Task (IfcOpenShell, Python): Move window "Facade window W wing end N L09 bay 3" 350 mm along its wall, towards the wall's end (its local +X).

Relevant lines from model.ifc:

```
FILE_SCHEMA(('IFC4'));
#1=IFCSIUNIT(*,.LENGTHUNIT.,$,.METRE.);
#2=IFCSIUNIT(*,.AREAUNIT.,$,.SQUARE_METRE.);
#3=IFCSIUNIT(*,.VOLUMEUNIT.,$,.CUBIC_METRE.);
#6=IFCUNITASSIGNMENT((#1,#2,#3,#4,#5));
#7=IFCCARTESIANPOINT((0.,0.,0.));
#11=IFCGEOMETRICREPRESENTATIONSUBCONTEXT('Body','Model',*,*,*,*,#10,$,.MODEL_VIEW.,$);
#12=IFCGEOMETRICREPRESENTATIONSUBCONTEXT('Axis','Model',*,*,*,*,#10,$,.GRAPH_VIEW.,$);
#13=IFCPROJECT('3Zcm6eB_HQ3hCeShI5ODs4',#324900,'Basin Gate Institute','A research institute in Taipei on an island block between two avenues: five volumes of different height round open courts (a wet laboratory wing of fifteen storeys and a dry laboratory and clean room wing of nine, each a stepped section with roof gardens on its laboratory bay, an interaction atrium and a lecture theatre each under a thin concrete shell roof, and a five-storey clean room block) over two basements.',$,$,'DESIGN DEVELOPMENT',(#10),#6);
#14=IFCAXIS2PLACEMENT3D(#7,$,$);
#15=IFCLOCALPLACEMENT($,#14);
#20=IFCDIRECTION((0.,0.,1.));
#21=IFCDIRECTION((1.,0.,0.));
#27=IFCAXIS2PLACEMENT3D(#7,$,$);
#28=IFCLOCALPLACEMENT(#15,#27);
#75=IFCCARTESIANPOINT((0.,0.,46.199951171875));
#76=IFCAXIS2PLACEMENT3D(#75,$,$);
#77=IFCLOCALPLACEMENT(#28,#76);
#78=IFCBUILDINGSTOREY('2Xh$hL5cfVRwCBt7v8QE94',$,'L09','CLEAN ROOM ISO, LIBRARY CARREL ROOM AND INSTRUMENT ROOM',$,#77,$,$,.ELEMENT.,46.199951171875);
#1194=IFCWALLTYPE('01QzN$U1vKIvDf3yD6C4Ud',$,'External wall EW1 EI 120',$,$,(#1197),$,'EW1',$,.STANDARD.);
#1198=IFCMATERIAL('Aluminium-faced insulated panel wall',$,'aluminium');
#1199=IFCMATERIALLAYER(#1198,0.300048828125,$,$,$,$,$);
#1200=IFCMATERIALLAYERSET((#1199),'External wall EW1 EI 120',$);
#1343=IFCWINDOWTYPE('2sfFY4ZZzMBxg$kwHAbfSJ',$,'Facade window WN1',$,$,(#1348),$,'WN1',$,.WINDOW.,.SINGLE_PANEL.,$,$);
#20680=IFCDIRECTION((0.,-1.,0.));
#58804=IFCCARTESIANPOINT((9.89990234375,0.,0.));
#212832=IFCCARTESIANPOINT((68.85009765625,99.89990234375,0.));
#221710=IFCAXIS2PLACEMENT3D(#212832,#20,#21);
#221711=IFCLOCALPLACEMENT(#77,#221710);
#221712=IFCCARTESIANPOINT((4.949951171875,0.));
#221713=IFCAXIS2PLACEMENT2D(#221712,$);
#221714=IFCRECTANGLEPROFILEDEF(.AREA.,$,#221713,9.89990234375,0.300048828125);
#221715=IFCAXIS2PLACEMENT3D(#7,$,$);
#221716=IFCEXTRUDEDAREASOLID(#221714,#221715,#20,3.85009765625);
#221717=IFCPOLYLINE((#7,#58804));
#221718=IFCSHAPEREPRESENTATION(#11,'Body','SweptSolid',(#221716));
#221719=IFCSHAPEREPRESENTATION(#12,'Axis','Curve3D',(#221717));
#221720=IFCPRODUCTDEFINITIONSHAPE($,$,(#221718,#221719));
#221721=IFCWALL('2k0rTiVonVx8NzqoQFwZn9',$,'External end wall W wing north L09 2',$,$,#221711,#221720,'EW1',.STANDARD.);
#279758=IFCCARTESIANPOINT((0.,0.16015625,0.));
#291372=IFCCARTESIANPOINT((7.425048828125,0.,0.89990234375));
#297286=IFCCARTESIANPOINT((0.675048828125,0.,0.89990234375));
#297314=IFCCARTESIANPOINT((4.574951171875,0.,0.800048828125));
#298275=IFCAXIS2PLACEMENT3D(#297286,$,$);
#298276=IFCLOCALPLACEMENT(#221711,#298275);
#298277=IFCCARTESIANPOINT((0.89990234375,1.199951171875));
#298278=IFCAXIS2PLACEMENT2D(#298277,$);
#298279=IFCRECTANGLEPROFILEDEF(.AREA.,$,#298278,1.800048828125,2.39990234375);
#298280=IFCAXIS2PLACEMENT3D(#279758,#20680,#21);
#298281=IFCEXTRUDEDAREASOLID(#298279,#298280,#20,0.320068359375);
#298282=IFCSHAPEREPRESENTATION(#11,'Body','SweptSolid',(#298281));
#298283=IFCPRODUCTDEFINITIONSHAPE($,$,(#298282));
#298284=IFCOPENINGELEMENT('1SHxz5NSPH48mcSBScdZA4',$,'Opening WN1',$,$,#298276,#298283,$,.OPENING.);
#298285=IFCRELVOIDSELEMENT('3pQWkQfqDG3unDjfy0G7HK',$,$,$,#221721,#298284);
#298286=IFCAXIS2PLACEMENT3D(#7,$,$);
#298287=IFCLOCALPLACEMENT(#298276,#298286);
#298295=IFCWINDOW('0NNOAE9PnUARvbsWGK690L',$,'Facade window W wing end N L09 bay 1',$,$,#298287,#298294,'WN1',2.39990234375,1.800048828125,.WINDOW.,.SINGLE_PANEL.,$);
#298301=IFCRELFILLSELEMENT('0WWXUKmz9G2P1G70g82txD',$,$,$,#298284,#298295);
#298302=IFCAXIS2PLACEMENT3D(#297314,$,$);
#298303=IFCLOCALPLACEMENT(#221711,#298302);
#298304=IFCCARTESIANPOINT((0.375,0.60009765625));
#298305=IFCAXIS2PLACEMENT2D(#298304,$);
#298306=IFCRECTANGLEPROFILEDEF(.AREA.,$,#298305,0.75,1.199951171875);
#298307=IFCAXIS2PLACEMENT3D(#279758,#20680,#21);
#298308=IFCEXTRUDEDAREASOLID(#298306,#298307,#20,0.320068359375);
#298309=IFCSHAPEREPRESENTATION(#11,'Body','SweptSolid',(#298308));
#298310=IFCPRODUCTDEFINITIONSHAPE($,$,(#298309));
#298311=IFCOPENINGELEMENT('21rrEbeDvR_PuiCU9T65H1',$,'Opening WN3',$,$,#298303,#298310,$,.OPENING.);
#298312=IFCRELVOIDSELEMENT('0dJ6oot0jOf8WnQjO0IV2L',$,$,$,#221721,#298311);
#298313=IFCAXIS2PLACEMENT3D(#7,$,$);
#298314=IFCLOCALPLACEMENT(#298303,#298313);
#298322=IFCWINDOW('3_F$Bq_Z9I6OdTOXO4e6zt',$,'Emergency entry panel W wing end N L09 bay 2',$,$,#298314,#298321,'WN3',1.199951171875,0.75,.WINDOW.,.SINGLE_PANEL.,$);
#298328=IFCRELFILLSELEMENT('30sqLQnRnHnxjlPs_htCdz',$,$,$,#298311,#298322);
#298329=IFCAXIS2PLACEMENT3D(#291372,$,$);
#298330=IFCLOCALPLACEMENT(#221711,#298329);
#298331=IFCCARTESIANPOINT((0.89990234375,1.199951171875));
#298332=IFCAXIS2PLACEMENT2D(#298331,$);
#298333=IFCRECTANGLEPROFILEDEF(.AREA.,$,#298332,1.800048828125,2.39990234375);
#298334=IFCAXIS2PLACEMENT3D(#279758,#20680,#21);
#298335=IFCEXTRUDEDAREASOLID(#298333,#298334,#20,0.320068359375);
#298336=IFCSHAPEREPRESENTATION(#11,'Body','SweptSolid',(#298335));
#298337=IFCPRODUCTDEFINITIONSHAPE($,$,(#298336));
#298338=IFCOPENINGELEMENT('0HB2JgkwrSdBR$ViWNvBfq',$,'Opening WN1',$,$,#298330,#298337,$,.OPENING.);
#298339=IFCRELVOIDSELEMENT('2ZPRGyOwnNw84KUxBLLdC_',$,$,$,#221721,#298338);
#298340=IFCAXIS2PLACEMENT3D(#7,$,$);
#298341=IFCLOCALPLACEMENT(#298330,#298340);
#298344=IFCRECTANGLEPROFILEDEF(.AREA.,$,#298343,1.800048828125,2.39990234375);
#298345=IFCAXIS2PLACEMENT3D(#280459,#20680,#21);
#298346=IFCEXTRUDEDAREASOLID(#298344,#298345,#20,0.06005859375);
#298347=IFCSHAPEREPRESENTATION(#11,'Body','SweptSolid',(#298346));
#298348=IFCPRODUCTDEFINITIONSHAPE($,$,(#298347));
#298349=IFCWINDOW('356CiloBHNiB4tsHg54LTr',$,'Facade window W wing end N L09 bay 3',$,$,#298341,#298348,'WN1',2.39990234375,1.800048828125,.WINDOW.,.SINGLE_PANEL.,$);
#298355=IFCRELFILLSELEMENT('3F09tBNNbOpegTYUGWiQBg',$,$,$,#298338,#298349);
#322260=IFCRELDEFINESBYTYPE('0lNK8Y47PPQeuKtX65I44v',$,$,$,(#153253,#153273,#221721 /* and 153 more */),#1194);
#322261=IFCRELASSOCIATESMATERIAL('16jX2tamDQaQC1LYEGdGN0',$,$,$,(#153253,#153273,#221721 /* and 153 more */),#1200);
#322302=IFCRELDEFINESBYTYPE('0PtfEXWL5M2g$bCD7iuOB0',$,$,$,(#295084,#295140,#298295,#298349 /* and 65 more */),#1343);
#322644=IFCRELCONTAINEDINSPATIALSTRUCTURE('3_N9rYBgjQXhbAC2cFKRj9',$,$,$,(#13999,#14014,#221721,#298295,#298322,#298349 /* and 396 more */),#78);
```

```python
import ifcopenshell
import ifcopenshell.api.geometry
import ifcopenshell.util.placement

model = ifcopenshell.open("model.ifc")

window = model.by_guid("356CiloBHNiB4tsHg54LTr")
opening = window.FillsVoids[0].RelatingOpeningElement
wall = opening.VoidsElements[0].RelatingBuildingElement

wall_matrix = ifcopenshell.util.placement.get_local_placement(wall.ObjectPlacement)
shift = wall_matrix[:3, 0] * 0.35
before = ifcopenshell.util.placement.get_local_placement(window.ObjectPlacement)[:3, 3].copy()

# The window is placed relative to its opening, so it follows when the opening moves.
matrix = ifcopenshell.util.placement.get_local_placement(opening.ObjectPlacement)
matrix[:3, 3] += shift
ifcopenshell.api.geometry.edit_object_placement(
    model, product=opening, matrix=matrix, is_si=False, should_transform_children=True
)

after = ifcopenshell.util.placement.get_local_placement(window.ObjectPlacement)[:3, 3]
print("window moved by", (after - before).round(3) + 0.0)

model.write("model_v2.ifc")
```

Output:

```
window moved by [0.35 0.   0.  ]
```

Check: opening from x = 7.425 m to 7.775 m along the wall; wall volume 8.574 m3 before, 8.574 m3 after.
